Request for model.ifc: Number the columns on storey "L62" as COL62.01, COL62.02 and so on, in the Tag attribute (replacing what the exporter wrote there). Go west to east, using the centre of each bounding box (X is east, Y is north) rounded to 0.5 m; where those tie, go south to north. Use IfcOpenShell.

First a look at what the model holds.

```python
import ifcopenshell
import ifcopenshell.util.element
import ifcopenshell.util.placement

model = ifcopenshell.open("model.ifc")
print(model.schema)
storey = next(s for s in model.by_type("IfcBuildingStorey") if s.Name == "L62")
columns = [e for e in ifcopenshell.util.element.get_decomposition(storey) if e.is_a("IfcColumn")]
for e in sorted(columns, key=lambda e: e.id()):
    origin = ifcopenshell.util.placement.get_local_placement(e.ObjectPlacement)[:3, 3]
    print(e.id(), e.Tag, e.Name, origin.round(2) + 0.0, sep=" | ")
```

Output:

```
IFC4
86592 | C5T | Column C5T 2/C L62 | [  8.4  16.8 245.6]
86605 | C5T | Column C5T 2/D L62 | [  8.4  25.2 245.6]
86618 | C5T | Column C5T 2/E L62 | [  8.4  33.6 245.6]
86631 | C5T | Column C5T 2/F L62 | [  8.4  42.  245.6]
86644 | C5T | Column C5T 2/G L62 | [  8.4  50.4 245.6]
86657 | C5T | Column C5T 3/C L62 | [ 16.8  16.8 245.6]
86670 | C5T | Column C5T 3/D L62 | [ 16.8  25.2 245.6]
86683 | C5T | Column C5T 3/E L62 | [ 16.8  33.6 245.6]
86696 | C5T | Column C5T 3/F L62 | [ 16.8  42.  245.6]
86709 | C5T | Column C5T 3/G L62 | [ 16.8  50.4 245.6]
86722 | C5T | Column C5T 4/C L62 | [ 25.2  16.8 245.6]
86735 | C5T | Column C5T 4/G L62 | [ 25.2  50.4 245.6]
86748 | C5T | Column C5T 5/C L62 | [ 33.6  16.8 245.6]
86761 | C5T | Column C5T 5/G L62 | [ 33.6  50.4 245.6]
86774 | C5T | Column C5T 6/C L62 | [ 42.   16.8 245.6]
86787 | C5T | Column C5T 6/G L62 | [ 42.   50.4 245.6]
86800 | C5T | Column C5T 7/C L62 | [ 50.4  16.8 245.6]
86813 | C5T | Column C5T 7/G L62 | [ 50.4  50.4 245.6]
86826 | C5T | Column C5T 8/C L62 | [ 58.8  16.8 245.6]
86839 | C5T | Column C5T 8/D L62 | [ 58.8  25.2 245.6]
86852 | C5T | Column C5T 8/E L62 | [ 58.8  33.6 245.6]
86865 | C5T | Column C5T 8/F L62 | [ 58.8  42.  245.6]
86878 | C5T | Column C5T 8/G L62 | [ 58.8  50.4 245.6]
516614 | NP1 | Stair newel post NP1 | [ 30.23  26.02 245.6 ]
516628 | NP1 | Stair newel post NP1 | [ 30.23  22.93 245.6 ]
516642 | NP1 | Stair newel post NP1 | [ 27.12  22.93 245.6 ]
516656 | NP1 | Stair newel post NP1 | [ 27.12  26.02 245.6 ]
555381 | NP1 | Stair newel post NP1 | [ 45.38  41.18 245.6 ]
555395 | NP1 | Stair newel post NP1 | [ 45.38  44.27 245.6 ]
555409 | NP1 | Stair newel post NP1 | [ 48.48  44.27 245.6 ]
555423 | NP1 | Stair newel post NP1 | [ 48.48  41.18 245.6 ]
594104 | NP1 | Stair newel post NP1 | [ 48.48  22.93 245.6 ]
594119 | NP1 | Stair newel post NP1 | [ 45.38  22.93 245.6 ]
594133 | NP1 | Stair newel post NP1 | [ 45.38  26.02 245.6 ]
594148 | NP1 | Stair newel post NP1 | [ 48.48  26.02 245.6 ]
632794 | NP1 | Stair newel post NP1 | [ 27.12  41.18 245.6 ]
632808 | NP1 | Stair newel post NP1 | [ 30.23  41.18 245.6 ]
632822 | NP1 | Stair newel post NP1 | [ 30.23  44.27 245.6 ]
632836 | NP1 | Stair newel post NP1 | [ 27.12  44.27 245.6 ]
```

```python
import ifcopenshell
import ifcopenshell.geom
import ifcopenshell.util.element
import ifcopenshell.util.shape

model = ifcopenshell.open("model.ifc")
settings = ifcopenshell.geom.settings()
settings.set("use-world-coords", True)


def centre(element):
    shape = ifcopenshell.geom.create_shape(settings, element)
    return ifcopenshell.util.shape.get_bbox_centroid(shape.geometry)


storey = next(s for s in model.by_type("IfcBuildingStorey") if s.Name == "L62")
columns = [e for e in ifcopenshell.util.element.get_decomposition(storey) if e.is_a("IfcColumn")]

# Insertion points can sit at a corner or the storey origin, so sort by the geometry (in metres).
centres = {e: centre(e) for e in columns}
columns.sort(key=lambda e: (round(centres[e][0] / 0.5), centres[e][1]))

for i, e in enumerate(columns, start=1):
    number = f"COL62.{i:02d}"
    e.Tag = number
    print(e.id(), number)

model.write("model_updated.ifc")
```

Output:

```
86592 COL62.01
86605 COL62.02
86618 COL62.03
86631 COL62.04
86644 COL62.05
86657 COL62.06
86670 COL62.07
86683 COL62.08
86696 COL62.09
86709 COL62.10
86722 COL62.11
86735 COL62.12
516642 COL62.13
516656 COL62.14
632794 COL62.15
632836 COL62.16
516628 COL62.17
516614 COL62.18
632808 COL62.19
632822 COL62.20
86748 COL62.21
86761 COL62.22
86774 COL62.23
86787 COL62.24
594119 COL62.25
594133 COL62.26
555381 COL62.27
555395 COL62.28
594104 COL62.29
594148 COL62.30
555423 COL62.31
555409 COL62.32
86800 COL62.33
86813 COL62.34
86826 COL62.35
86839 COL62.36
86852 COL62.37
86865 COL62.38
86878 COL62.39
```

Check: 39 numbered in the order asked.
